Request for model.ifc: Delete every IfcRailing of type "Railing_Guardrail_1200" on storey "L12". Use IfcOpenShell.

First a look at what the model holds.

```python
import ifcopenshell
import ifcopenshell.util.element

model = ifcopenshell.open("model.ifc")
print(model.schema)
storey = next(s for s in model.by_type("IfcBuildingStorey") if s.Name == "L12")
railings = [e for e in ifcopenshell.util.element.get_decomposition(storey) if e.is_a("IfcRailing")]
seen = {}
for e in railings:
    element_type = ifcopenshell.util.element.get_type(e)
    name = element_type.Name if element_type not in (None, e) else None
    seen[name] = seen.get(name, 0) + 1
for name, count in sorted(seen.items(), key=str):
    print(count, "x", name)
```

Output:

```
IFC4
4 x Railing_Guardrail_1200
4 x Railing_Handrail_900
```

```python
import ifcopenshell
import ifcopenshell.api.root
import ifcopenshell.util.element

model = ifcopenshell.open("model.ifc")

storey = next(s for s in model.by_type("IfcBuildingStorey") if s.Name == "L12")
railings = [e for e in ifcopenshell.util.element.get_decomposition(storey) if e.is_a("IfcRailing")]
targets = [e for e in railings if (t := ifcopenshell.util.element.get_type(e)) not in (None, e) and t.Name == "Railing_Guardrail_1200"]

for e in targets:
    ifcopenshell.api.root.remove_product(model, product=e)
print(len(targets), "removed")

model.write("model_updated.ifc")
```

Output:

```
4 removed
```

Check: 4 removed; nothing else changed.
